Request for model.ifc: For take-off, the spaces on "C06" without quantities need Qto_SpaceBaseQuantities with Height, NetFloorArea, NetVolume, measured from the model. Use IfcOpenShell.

First a look at what the model holds.

```python
import ifcopenshell
import ifcopenshell.util.element
import ifcopenshell.util.unit

model = ifcopenshell.open("model.ifc")
print(model.schema)
for unit_type in ("LENGTHUNIT", "AREAUNIT", "VOLUMEUNIT"):
    print(unit_type, ifcopenshell.util.unit.calculate_unit_scale(model, unit_type))
storey = next(s for s in model.by_type("IfcBuildingStorey") if s.Name == "C06")
spaces = [e for e in ifcopenshell.util.element.get_decomposition(storey) if e.is_a("IfcSpace")]
for e in sorted(spaces, key=lambda e: e.id()):
    print(e.id(), e.is_a(), e.Name, list(ifcopenshell.util.element.get_psets(e, qtos_only=True)), sep=" | ")
```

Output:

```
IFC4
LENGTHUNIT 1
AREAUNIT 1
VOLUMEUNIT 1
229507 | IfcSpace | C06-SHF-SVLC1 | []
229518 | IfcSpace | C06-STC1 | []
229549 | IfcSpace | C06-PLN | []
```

```python
import ifcopenshell
import ifcopenshell.api.pset
import ifcopenshell.geom
import ifcopenshell.util.element
import ifcopenshell.util.shape
import ifcopenshell.util.unit

model = ifcopenshell.open("model.ifc")
unit_scale = ifcopenshell.util.unit.calculate_unit_scale(model)
area_scale = ifcopenshell.util.unit.calculate_unit_scale(model, "AREAUNIT")
volume_scale = ifcopenshell.util.unit.calculate_unit_scale(model, "VOLUMEUNIT")
settings = ifcopenshell.geom.settings()

storey = next(s for s in model.by_type("IfcBuildingStorey") if s.Name == "C06")
spaces = [e for e in ifcopenshell.util.element.get_decomposition(storey) if e.is_a("IfcSpace")]

for e in sorted(spaces, key=lambda e: e.id()):
    if ifcopenshell.util.element.get_psets(e, qtos_only=True, should_inherit=False):
        continue
    # Geometry comes back in metres, in the element's own axes.
    shape = ifcopenshell.geom.create_shape(settings, e)
    values = {
        "Height": ifcopenshell.util.shape.get_z(shape.geometry) / unit_scale,
        "NetFloorArea": ifcopenshell.util.shape.get_footprint_area(shape.geometry) / area_scale,
        "NetVolume": ifcopenshell.util.shape.get_volume(shape.geometry) / volume_scale,
    }
    qto = ifcopenshell.api.pset.add_qto(model, product=e, name="Qto_SpaceBaseQuantities")
    ifcopenshell.api.pset.edit_qto(model, qto=qto, properties=values)
    print(e.id(), {k: round(v, 3) for k, v in values.items()})

model.write("model-out.ifc")
```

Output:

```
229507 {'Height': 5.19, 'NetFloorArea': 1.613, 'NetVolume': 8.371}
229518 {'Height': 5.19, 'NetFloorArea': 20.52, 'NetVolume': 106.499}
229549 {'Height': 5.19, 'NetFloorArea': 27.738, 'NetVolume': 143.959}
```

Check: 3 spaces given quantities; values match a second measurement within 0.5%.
